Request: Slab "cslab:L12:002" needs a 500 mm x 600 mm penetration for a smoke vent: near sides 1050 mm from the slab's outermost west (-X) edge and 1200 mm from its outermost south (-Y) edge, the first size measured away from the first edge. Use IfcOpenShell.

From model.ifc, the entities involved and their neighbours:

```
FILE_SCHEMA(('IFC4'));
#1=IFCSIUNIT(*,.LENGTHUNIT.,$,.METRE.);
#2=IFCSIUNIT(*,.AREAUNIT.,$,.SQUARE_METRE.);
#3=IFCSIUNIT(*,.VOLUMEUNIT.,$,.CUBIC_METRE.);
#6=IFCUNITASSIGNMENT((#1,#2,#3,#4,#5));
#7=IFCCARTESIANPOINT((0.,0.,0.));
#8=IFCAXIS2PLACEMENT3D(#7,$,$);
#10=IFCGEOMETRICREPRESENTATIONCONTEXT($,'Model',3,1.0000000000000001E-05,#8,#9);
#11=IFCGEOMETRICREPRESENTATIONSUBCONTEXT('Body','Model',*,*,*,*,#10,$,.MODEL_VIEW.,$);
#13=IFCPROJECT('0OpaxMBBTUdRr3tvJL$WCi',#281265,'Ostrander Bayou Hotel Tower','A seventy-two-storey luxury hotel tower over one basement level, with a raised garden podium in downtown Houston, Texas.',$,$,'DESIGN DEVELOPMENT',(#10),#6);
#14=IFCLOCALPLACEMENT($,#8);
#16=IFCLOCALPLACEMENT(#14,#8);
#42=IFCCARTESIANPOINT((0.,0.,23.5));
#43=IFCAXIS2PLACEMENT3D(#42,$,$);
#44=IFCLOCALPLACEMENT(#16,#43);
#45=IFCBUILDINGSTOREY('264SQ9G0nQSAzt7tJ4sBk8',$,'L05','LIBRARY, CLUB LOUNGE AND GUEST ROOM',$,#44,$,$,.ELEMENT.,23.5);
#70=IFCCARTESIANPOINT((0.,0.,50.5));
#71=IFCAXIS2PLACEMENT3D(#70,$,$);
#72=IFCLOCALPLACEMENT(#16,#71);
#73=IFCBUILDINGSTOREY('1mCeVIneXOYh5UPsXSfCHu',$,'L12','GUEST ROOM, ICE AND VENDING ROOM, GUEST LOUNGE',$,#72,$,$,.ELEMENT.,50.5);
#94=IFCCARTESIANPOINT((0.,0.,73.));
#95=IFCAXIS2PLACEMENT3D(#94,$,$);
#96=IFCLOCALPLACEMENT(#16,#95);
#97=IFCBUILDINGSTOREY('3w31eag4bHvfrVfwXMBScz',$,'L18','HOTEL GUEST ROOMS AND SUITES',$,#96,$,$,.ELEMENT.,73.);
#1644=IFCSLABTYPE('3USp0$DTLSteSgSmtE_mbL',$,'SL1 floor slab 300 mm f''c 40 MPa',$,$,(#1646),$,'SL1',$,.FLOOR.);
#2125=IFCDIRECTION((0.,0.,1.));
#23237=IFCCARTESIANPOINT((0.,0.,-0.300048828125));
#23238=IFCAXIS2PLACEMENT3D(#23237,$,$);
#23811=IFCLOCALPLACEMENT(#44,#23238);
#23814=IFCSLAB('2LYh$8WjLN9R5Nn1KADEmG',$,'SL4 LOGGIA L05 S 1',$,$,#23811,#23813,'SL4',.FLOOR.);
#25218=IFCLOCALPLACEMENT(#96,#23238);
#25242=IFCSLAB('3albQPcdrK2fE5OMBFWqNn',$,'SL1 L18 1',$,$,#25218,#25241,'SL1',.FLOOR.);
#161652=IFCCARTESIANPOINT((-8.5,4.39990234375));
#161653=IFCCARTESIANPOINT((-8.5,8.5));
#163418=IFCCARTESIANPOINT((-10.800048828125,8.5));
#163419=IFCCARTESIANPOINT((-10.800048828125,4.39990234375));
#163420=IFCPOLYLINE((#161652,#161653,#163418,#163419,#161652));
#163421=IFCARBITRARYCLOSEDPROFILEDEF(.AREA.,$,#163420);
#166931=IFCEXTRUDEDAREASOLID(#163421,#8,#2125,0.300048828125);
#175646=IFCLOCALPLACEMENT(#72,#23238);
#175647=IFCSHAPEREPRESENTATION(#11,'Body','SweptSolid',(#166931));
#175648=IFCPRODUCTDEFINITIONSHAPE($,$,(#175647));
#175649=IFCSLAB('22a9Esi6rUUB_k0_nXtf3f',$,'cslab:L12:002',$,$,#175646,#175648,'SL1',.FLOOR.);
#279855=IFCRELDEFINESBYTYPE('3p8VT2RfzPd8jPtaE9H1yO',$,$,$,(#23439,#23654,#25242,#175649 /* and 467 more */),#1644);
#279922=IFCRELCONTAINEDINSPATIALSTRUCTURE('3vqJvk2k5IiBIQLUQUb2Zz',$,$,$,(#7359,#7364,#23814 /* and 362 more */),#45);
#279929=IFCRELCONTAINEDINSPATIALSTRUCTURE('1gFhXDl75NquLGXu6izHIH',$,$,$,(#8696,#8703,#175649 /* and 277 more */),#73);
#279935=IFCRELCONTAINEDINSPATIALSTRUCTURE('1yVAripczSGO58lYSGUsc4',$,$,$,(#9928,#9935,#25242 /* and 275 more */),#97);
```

```python
import numpy as np
import ifcopenshell
import ifcopenshell.api.feature
import ifcopenshell.api.geometry
import ifcopenshell.api.root
import ifcopenshell.geom
import ifcopenshell.util.placement
import ifcopenshell.util.representation
import ifcopenshell.util.shape
import ifcopenshell.util.unit

model = ifcopenshell.open("model.ifc")
unit_scale = ifcopenshell.util.unit.calculate_unit_scale(model)
settings = ifcopenshell.geom.settings()


def volume(element):
    """Net volume in cubic metres, openings subtracted."""
    shape = ifcopenshell.geom.create_shape(settings, element)
    return ifcopenshell.util.shape.get_volume(shape.geometry)


slab = model.by_guid("22a9Esi6rUUB_k0_nXtf3f")
before = volume(slab)

# Extent in the slab's own axes, in metres. The edges named are its -X and -Y sides.
slab_shape = ifcopenshell.geom.create_shape(settings, slab)
vertices = ifcopenshell.util.shape.get_vertices(slab_shape.geometry)
x_min, y_min, bottom = vertices.min(axis=0)
top = vertices[:, 2].max()

opening = ifcopenshell.api.root.create_entity(model, ifc_class="IfcOpeningElement", name="Smoke vent opening", predefined_type="OPENING")
context = ifcopenshell.util.representation.get_context(model, "Model", "Body", "MODEL_VIEW")
width, depth = 0.5, 0.6
outline = [(0.0, 0.0), (width, 0.0), (width, depth), (0.0, depth), (0.0, 0.0)]
# Overshoot both faces by 50 mm so the cut is clean.
shape = ifcopenshell.api.geometry.add_slab_representation(
    model, context=context, depth=top - bottom + 0.1, polyline=outline
)
ifcopenshell.api.geometry.assign_representation(model, product=opening, representation=shape)

matrix = ifcopenshell.util.placement.get_local_placement(slab.ObjectPlacement)
matrix[:, 3] = matrix @ np.append(np.array([x_min + 1.05, y_min + 1.2, bottom - 0.05]) / unit_scale, 1.0)
ifcopenshell.api.geometry.edit_object_placement(model, product=opening, matrix=matrix, is_si=False)
ifcopenshell.api.feature.add_feature(model, feature=opening, element=slab)

after = volume(slab)

print(f"slab volume {before:.3f} -> {after:.3f} m3")

model.write("model-out.ifc")
```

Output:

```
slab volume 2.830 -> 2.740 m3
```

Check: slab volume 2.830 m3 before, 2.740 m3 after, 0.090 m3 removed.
